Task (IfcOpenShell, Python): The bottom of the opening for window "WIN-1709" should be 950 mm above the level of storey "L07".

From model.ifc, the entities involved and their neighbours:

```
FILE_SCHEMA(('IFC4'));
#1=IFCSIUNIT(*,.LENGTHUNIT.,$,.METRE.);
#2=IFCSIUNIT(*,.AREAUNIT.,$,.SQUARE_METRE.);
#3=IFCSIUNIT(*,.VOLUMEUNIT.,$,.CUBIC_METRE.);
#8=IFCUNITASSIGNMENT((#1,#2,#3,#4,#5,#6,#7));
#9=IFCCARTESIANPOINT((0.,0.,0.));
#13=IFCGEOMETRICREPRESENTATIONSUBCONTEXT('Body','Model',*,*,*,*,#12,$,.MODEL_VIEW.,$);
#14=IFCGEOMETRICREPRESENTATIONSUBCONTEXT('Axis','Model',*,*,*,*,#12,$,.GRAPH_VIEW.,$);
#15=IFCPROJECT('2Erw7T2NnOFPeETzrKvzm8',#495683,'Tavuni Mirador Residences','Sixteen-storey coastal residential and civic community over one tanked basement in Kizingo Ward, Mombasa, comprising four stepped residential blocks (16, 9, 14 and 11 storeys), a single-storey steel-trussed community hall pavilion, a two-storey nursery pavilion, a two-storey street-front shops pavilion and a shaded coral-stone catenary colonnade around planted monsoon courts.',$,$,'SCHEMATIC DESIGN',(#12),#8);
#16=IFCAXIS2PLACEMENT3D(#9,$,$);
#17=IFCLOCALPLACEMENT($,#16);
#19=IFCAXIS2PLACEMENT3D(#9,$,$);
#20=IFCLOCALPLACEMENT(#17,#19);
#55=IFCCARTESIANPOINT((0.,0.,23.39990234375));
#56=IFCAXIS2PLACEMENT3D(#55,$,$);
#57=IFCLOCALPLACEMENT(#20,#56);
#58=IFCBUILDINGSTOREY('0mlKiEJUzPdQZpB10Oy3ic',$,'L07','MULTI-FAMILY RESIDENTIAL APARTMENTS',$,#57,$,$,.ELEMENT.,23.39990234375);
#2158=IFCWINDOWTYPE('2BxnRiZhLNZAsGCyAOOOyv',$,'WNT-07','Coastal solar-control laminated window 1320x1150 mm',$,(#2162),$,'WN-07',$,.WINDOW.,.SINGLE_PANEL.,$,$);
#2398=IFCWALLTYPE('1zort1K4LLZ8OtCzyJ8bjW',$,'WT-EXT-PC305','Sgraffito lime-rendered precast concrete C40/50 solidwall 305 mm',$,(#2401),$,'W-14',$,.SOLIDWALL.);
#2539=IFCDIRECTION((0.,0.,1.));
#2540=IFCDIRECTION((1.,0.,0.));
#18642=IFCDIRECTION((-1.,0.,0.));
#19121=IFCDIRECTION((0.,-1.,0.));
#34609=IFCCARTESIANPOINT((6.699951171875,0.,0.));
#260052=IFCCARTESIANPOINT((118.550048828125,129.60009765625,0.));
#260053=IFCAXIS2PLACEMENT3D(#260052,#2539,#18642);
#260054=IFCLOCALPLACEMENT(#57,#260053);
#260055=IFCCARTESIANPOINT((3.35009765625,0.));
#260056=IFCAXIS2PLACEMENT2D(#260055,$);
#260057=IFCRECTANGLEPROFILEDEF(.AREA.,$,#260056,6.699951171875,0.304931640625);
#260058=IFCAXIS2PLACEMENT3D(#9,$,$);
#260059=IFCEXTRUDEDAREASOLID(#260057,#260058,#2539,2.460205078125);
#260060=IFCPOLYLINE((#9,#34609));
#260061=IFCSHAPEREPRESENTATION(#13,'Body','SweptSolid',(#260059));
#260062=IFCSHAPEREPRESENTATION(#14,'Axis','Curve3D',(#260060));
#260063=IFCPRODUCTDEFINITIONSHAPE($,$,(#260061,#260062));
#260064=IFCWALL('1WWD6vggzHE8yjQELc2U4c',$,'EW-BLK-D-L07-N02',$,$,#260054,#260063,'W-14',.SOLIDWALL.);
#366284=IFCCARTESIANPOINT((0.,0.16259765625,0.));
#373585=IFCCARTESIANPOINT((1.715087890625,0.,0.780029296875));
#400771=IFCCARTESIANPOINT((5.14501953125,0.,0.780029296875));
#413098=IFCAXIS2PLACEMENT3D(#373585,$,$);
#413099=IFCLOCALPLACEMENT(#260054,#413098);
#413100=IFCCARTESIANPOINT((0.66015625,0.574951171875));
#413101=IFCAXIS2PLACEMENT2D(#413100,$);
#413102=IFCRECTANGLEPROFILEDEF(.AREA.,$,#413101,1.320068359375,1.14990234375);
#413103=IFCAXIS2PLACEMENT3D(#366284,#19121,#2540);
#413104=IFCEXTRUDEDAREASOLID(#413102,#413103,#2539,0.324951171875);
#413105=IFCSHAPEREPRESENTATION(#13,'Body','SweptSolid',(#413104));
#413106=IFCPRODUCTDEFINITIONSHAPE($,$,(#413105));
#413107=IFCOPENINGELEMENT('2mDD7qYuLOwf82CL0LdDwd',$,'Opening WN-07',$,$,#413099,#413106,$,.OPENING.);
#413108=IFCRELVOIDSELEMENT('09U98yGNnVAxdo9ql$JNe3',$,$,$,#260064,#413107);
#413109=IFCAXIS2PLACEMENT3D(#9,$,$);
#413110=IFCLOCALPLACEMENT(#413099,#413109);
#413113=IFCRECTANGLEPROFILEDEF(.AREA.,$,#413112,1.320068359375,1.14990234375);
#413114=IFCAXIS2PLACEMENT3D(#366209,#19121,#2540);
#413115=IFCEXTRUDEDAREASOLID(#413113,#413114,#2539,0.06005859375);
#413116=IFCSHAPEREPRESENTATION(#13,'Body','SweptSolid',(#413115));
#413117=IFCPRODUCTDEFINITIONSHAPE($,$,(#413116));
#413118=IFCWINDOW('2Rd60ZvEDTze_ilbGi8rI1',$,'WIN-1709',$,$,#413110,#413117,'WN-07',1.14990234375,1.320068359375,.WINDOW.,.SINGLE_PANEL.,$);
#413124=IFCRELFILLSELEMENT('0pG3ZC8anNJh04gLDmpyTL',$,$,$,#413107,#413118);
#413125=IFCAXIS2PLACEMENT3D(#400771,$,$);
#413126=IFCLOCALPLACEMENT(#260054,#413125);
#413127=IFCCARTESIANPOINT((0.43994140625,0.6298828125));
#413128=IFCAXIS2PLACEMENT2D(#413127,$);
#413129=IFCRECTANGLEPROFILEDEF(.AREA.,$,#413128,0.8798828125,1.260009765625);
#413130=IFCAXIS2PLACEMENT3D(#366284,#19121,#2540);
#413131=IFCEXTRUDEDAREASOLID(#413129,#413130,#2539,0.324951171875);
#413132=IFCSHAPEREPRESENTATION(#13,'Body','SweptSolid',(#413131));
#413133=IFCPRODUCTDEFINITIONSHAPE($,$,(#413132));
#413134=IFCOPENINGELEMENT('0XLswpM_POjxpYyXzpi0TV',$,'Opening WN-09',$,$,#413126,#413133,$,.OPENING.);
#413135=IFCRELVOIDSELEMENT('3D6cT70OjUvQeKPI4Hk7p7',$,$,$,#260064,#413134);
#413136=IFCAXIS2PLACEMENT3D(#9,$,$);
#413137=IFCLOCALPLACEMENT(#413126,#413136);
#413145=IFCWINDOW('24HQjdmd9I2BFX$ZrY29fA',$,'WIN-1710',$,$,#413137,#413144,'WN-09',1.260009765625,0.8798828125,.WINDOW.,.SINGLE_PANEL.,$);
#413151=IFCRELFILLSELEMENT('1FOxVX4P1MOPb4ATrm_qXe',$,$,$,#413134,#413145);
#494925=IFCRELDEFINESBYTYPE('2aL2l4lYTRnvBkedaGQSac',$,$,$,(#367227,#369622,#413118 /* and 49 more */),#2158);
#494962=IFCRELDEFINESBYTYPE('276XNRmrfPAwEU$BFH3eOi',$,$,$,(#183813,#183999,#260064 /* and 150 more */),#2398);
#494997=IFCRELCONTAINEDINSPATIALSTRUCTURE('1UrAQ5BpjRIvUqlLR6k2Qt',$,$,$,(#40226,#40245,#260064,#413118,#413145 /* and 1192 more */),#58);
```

```python
import numpy as np
import ifcopenshell
import ifcopenshell.api.geometry
import ifcopenshell.geom
import ifcopenshell.util.element
import ifcopenshell.util.placement
import ifcopenshell.util.shape
import ifcopenshell.util.unit

model = ifcopenshell.open("model.ifc")
unit_scale = ifcopenshell.util.unit.calculate_unit_scale(model)

window = model.by_id(413118)
opening = window.FillsVoids[0].RelatingOpeningElement
storey = ifcopenshell.util.element.get_container(window, ifc_class="IfcBuildingStorey")
level = ifcopenshell.util.placement.get_local_placement(storey.ObjectPlacement)[2, 3]

# The opening's origin need not be at the sill, so measure its lowest point.
shape = ifcopenshell.geom.create_shape(ifcopenshell.geom.settings(), opening)
bottom = ifcopenshell.util.shape.get_shape_bottom_elevation(shape, shape.geometry) / unit_scale
dz = level + 0.95 / unit_scale - bottom

shift = np.array([0.0, 0.0, dz])
# The window is placed relative to its opening, so it follows when the opening moves.
matrix = ifcopenshell.util.placement.get_local_placement(opening.ObjectPlacement)
matrix[:3, 3] += shift
ifcopenshell.api.geometry.edit_object_placement(
    model, product=opening, matrix=matrix, is_si=False, should_transform_children=True
)

print(f"moved by {dz * unit_scale:+.3f} m")

model.write("model_updated.ifc")
```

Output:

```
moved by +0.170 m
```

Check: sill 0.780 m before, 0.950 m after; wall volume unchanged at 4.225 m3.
